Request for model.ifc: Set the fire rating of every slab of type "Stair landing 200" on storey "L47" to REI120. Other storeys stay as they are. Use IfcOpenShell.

First a look at what the model holds.

```python
import ifcopenshell
import ifcopenshell.util.element

model = ifcopenshell.open("model.ifc")
print(model.schema)
storey = next(s for s in model.by_type("IfcBuildingStorey") if s.Name == "L47")
slabs = [e for e in ifcopenshell.util.element.get_decomposition(storey) if e.is_a("IfcSlab")]
seen = {}
for e in slabs:
    element_type = ifcopenshell.util.element.get_type(e)
    key = (element_type.Name if element_type != e and element_type else None, ifcopenshell.util.element.get_pset(e, "Pset_SlabCommon", "FireRating"))
    seen[key] = seen.get(key, 0) + 1
for (name, value), count in sorted(seen.items(), key=str):
    print(count, "x", name, "|", value)
```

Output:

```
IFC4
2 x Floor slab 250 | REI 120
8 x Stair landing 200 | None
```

```python
import ifcopenshell
import ifcopenshell.api.pset
import ifcopenshell.util.element

model = ifcopenshell.open("model.ifc")

storey = next(s for s in model.by_type("IfcBuildingStorey") if s.Name == "L47")
slabs = [e for e in ifcopenshell.util.element.get_decomposition(storey) if e.is_a("IfcSlab")]

count = 0
for e in slabs:
    element_type = ifcopenshell.util.element.get_type(e)
    if element_type in (None, e) or element_type.Name != "Stair landing 200":
        continue
    found = ifcopenshell.util.element.get_pset(e, "Pset_SlabCommon", should_inherit=False)
    if found:
        pset = model.by_id(found["id"])
        if len(ifcopenshell.util.element.get_elements_by_pset(pset)) > 1:
            pset = ifcopenshell.api.pset.unshare_pset(model, products=[e], pset=pset)[0]
    else:
        pset = ifcopenshell.api.pset.add_pset(model, product=e, name="Pset_SlabCommon")
    ifcopenshell.api.pset.edit_pset(model, pset=pset, properties={"FireRating": "REI120"})
    count += 1

print(count, "slabs updated")

model.write("model-out.ifc")
```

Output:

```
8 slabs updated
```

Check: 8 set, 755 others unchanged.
